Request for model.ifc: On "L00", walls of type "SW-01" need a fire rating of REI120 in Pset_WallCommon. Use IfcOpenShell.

First a look at what the model holds.

```python
import ifcopenshell
import ifcopenshell.util.element

model = ifcopenshell.open("model.ifc")
print(model.schema)
storey = next(s for s in model.by_type("IfcBuildingStorey") if s.Name == "L00")
walls = [e for e in ifcopenshell.util.element.get_decomposition(storey) if e.is_a("IfcWall")]
seen = {}
for e in walls:
    element_type = ifcopenshell.util.element.get_type(e)
    key = (element_type.Name if element_type != e and element_type else None, ifcopenshell.util.element.get_pset(e, "Pset_WallCommon", "FireRating"))
    seen[key] = seen.get(key, 0) + 1
for (name, value), count in sorted(seen.items(), key=str):
    print(count, "x", name, "|", value)
```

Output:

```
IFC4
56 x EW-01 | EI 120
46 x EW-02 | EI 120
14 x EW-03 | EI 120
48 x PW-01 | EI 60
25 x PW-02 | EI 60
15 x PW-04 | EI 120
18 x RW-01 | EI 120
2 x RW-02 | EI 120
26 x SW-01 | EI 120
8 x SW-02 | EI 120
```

```python
import ifcopenshell
import ifcopenshell.api.pset
import ifcopenshell.util.element

model = ifcopenshell.open("model.ifc")

storey = next(s for s in model.by_type("IfcBuildingStorey") if s.Name == "L00")
walls = [e for e in ifcopenshell.util.element.get_decomposition(storey) if e.is_a("IfcWall")]

count = 0
for e in walls:
    element_type = ifcopenshell.util.element.get_type(e)
    if element_type in (None, e) or element_type.Name != "SW-01":
        continue
    # add_pset returns the element's existing set when there is one.
    pset = ifcopenshell.api.pset.add_pset(model, product=e, name="Pset_WallCommon")
    ifcopenshell.api.pset.edit_pset(model, pset=pset, properties={"FireRating": "REI120"})
    count += 1

print(count, "walls updated")

model.write("model-out.ifc")
```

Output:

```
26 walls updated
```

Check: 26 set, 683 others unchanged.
